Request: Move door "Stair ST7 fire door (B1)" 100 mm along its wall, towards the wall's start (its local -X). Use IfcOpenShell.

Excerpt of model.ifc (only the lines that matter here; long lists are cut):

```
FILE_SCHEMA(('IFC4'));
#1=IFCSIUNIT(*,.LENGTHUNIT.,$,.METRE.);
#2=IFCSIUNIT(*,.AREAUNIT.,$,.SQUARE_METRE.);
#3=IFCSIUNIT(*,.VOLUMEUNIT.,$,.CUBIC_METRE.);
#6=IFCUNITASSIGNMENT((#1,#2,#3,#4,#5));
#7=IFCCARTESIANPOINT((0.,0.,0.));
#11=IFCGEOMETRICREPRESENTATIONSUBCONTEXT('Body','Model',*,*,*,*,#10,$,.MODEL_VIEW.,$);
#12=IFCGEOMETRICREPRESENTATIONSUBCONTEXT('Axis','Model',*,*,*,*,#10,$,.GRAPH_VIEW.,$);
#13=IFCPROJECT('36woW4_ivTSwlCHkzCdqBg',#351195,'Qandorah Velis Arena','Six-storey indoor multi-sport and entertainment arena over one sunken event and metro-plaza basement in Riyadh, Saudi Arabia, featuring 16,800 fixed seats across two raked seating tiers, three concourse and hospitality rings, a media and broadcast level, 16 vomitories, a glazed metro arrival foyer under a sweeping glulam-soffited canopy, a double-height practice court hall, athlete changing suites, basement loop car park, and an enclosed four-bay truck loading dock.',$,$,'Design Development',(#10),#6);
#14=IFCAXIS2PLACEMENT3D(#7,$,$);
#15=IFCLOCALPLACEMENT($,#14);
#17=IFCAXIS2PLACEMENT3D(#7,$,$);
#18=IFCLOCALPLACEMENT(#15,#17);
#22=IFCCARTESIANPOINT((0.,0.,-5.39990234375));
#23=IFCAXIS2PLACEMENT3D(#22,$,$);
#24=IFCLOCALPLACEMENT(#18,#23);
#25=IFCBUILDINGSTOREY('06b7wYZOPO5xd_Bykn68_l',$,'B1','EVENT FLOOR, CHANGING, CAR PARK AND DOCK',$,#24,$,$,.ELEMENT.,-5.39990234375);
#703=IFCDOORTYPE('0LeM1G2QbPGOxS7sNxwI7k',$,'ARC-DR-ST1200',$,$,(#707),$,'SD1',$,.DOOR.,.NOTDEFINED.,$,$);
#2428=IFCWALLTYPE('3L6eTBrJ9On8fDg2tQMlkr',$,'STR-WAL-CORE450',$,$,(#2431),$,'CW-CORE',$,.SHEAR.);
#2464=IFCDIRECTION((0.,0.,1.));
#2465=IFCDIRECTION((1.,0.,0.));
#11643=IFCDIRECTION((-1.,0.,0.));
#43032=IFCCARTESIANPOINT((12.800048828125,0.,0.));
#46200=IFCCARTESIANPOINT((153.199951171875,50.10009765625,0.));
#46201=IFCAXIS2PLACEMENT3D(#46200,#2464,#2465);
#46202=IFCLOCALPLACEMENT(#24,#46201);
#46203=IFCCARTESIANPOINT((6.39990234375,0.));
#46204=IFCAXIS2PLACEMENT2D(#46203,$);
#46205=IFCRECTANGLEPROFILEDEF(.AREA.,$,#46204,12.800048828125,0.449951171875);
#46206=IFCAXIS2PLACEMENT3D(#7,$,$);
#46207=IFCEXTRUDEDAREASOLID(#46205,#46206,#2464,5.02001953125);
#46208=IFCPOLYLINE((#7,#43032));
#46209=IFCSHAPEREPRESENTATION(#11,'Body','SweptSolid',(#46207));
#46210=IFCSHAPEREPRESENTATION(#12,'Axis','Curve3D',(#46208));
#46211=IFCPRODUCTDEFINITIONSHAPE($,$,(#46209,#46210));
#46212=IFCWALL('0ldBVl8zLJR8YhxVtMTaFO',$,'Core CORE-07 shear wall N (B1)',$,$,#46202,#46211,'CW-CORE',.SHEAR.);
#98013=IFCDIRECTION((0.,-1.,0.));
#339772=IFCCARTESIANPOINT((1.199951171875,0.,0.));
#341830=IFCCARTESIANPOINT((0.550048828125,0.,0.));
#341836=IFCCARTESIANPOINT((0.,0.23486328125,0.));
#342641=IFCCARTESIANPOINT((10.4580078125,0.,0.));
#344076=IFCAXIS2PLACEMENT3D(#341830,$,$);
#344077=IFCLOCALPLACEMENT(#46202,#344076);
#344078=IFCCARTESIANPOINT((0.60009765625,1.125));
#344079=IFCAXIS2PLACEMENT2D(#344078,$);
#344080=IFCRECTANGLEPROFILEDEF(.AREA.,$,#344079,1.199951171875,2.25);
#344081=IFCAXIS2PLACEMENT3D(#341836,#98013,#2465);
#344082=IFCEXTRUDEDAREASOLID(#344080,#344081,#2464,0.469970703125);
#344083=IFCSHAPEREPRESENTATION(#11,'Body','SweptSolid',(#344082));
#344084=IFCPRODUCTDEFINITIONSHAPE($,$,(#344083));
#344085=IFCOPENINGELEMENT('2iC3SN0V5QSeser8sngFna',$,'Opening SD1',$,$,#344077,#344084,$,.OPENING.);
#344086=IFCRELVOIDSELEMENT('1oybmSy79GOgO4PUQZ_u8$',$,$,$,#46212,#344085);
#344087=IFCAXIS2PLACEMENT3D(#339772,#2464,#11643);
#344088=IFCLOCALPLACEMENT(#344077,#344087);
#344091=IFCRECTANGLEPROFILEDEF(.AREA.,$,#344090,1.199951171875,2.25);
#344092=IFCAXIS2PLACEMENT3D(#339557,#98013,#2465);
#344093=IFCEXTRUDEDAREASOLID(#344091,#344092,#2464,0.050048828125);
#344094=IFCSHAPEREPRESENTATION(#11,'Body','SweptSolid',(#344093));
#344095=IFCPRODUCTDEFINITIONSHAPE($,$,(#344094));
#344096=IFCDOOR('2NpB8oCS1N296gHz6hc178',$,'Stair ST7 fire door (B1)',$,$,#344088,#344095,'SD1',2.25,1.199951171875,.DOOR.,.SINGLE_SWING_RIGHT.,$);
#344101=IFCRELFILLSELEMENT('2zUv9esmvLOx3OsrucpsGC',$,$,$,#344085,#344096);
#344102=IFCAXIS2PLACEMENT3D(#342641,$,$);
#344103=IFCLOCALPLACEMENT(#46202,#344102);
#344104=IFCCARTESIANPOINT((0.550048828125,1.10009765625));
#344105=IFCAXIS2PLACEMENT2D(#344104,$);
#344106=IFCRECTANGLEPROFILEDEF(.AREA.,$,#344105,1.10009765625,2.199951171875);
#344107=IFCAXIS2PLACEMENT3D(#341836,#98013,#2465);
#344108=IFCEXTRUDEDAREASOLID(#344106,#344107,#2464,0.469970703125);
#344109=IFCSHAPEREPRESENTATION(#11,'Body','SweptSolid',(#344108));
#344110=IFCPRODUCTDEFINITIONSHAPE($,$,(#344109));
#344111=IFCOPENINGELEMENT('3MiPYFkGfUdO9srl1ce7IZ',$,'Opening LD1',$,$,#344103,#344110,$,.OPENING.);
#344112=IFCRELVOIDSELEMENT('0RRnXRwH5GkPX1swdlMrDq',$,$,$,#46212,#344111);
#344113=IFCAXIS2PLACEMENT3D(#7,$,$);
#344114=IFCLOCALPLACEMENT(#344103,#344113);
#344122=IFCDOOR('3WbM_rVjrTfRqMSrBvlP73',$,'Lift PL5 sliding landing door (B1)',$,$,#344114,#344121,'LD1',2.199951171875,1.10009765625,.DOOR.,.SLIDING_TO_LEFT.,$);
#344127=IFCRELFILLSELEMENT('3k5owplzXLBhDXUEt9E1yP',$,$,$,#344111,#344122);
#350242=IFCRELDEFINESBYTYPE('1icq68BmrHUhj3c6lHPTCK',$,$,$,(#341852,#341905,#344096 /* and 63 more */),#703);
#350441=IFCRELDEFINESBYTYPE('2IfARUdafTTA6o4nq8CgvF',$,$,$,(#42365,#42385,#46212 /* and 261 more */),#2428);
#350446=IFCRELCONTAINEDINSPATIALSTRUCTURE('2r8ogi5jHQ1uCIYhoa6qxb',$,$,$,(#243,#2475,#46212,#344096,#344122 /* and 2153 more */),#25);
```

```python
import ifcopenshell
import ifcopenshell.api.geometry
import ifcopenshell.util.placement
import ifcopenshell.util.unit

model = ifcopenshell.open("model.ifc")
unit_scale = ifcopenshell.util.unit.calculate_unit_scale(model)

door = model.by_id(344096)
opening = door.FillsVoids[0].RelatingOpeningElement
wall = opening.VoidsElements[0].RelatingBuildingElement

wall_matrix = ifcopenshell.util.placement.get_local_placement(wall.ObjectPlacement)
shift = wall_matrix[:3, 0] * -0.1 / unit_scale
before = ifcopenshell.util.placement.get_local_placement(door.ObjectPlacement)[:3, 3].copy()

# The door is placed relative to its opening, so it follows when the opening moves.
matrix = ifcopenshell.util.placement.get_local_placement(opening.ObjectPlacement)
matrix[:3, 3] += shift
ifcopenshell.api.geometry.edit_object_placement(
    model, product=opening, matrix=matrix, is_si=False, should_transform_children=True
)

after = ifcopenshell.util.placement.get_local_placement(door.ObjectPlacement)[:3, 3]
print("door moved by", (after - before).round(3) + 0.0)

model.write("model-out.ifc")
```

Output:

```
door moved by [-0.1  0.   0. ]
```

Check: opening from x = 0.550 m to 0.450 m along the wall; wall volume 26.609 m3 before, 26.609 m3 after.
